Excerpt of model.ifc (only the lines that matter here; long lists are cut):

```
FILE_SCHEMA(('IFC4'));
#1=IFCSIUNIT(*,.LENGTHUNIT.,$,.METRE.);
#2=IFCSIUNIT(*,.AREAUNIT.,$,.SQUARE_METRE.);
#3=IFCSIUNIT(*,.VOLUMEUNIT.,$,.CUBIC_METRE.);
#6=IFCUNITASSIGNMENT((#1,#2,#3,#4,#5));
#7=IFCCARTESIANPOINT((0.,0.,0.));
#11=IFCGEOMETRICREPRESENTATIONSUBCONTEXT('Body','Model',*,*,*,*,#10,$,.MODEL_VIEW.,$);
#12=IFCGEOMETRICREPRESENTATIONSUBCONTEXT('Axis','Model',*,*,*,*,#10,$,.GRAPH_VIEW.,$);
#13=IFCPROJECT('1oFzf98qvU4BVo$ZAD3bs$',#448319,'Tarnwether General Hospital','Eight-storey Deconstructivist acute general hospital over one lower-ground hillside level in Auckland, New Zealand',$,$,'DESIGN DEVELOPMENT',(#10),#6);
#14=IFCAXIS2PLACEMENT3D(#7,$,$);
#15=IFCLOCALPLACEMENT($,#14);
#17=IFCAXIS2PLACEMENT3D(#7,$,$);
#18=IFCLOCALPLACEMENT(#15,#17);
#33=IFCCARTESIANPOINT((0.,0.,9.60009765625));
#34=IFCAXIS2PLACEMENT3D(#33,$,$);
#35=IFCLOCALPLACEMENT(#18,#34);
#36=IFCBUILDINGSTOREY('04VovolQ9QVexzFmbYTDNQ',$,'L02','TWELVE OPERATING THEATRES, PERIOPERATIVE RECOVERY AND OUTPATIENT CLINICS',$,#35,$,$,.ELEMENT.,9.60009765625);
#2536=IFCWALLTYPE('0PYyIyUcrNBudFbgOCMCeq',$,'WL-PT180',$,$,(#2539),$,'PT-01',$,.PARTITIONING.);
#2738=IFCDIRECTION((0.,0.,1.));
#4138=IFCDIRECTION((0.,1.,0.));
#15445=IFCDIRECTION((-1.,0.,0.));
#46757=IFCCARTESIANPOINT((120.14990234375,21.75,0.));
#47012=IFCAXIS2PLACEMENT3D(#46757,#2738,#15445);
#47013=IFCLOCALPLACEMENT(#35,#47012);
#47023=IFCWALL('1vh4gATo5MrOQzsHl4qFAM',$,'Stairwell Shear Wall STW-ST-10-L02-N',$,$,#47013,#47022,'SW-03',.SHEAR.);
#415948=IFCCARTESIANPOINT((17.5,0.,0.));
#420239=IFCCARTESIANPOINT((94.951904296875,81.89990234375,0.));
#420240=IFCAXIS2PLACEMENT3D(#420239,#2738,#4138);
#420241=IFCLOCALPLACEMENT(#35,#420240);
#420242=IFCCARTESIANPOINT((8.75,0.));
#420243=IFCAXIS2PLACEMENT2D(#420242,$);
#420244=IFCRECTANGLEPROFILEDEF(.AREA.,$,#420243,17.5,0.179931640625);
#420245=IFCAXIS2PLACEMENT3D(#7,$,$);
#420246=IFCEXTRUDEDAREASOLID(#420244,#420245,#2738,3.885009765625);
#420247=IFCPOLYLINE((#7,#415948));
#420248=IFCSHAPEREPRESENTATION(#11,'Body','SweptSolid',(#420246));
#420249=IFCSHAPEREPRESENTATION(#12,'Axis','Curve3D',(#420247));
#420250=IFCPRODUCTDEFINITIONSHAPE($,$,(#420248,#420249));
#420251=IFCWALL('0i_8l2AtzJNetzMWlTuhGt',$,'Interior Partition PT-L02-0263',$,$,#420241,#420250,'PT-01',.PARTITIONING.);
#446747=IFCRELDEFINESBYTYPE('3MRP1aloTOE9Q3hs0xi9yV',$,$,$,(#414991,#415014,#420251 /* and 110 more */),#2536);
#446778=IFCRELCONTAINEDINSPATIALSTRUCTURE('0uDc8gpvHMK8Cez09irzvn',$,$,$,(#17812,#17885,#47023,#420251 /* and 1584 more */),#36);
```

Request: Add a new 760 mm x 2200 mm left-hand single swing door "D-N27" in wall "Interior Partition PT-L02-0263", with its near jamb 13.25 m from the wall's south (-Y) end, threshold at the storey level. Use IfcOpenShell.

```python
import numpy as np
import ifcopenshell
import ifcopenshell.api.feature
import ifcopenshell.api.geometry
import ifcopenshell.api.root
import ifcopenshell.api.spatial
import ifcopenshell.geom
import ifcopenshell.util.element
import ifcopenshell.util.placement
import ifcopenshell.util.representation
import ifcopenshell.util.shape
import ifcopenshell.util.unit

model = ifcopenshell.open("model.ifc")
unit_scale = ifcopenshell.util.unit.calculate_unit_scale(model)
settings = ifcopenshell.geom.settings()


def volume(element):
    """Net volume in cubic metres, openings subtracted."""
    shape = ifcopenshell.geom.create_shape(settings, element)
    return ifcopenshell.util.shape.get_volume(shape.geometry)


wall = model.by_guid("0i_8l2AtzJNetzMWlTuhGt")
storey = ifcopenshell.util.element.get_container(wall, ifc_class="IfcBuildingStorey")
context = ifcopenshell.util.representation.get_context(model, "Model", "Body", "MODEL_VIEW")
before = volume(wall)

width, height, from_end, sill = 0.76, 2.2, 13.25, 0.0  # metres

# The wall runs along its own X axis, and the end named is its -X end.
wall_shape = ifcopenshell.geom.create_shape(settings, wall)
x, y, z = ifcopenshell.util.shape.get_vertices(wall_shape.geometry).T
start = x.min() + from_end
face, thickness = float(y.min()), float(y.max() - y.min())
wall_matrix = ifcopenshell.util.placement.get_local_placement(wall.ObjectPlacement)
level = ifcopenshell.util.placement.get_local_placement(storey.ObjectPlacement)[2, 3]


def in_wall(x, y):
    """Placement at x, y metres in the wall's axes, at sill height."""
    matrix = wall_matrix.copy()
    matrix[:, 3] = wall_matrix @ np.array([x / unit_scale, y / unit_scale, 0.0, 1.0])
    matrix[2, 3] = level + sill / unit_scale
    return matrix


# Opening: a box that overshoots both wall faces by 50 mm.
opening = ifcopenshell.api.root.create_entity(model, ifc_class="IfcOpeningElement", predefined_type="OPENING")
box = ifcopenshell.api.geometry.add_wall_representation(
    model, context=context, length=width, height=height, thickness=thickness + 0.1
)
ifcopenshell.api.geometry.assign_representation(model, product=opening, representation=box)
ifcopenshell.api.geometry.edit_object_placement(model, product=opening, matrix=in_wall(start, face - 0.05), is_si=False)
ifcopenshell.api.feature.add_feature(model, feature=opening, element=wall)

door = ifcopenshell.api.root.create_entity(model, ifc_class="IfcDoor", name="D-N27", predefined_type="DOOR")
door.OverallWidth, door.OverallHeight = width / unit_scale, height / unit_scale
door.OperationType = "SINGLE_SWING_LEFT"
body = ifcopenshell.api.geometry.add_door_representation(
    model,
    context=context,
    overall_width=door.OverallWidth,
    overall_height=door.OverallHeight,
    operation_type="SINGLE_SWING_LEFT",
    lining_properties={"LiningDepth": thickness / unit_scale, "ThresholdDepth": thickness / unit_scale},
)
ifcopenshell.api.geometry.assign_representation(model, product=door, representation=body)
ifcopenshell.api.spatial.assign_container(model, products=[door], relating_structure=storey)
ifcopenshell.api.feature.add_filling(model, opening=opening, element=door)

# The lining spans the wall, so the door starts at the wall face.
ifcopenshell.api.geometry.edit_object_placement(model, product=door, matrix=in_wall(start, face), is_si=False)

after = volume(wall)

print(f"wall volume {before:.3f} -> {after:.3f} m3")

model.write("model_v2.ifc")
```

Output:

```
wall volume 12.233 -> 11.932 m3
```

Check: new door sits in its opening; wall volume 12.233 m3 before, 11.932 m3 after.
